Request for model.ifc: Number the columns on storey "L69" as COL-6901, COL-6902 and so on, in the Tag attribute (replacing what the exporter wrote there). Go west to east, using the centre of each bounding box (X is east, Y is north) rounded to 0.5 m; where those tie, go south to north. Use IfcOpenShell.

First a look at what the model holds.

```python
import ifcopenshell
import ifcopenshell.util.element
import ifcopenshell.util.placement

model = ifcopenshell.open("model.ifc")
print(model.schema)
storey = next(s for s in model.by_type("IfcBuildingStorey") if s.Name == "L69")
columns = [e for e in ifcopenshell.util.element.get_decomposition(storey) if e.is_a("IfcColumn")]
for e in sorted(columns, key=lambda e: e.id()):
    origin = ifcopenshell.util.placement.get_local_placement(e.ObjectPlacement)[:3, 3]
    print(e.id(), e.Tag, e.Name, origin.round(2) + 0.0, sep=" | ")
```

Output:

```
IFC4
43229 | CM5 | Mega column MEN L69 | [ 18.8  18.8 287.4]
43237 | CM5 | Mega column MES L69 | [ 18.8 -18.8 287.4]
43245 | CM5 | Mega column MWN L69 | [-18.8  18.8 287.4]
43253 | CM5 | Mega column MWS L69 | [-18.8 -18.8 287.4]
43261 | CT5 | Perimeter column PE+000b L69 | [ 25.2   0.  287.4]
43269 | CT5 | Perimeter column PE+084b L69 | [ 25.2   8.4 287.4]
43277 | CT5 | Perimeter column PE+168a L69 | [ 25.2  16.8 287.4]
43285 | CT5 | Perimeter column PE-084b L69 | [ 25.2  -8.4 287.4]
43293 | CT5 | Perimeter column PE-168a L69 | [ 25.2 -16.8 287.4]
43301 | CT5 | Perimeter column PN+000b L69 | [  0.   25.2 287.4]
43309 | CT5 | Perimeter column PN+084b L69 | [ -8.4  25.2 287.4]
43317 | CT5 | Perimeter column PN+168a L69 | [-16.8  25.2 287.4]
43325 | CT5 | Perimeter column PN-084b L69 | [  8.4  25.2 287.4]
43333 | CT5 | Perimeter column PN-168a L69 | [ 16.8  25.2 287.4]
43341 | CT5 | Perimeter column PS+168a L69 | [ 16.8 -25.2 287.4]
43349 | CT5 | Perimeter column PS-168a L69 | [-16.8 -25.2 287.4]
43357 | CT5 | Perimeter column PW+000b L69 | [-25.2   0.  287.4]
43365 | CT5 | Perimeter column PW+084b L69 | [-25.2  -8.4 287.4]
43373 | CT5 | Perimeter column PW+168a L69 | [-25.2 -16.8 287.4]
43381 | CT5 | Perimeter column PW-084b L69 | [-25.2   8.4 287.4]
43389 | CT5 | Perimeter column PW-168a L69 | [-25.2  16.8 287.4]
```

```python
import ifcopenshell
import ifcopenshell.geom
import ifcopenshell.util.element
import ifcopenshell.util.shape

model = ifcopenshell.open("model.ifc")
settings = ifcopenshell.geom.settings()
settings.set("use-world-coords", True)


def centre(element):
    shape = ifcopenshell.geom.create_shape(settings, element)
    return ifcopenshell.util.shape.get_bbox_centroid(shape.geometry)


storey = next(s for s in model.by_type("IfcBuildingStorey") if s.Name == "L69")
columns = [e for e in ifcopenshell.util.element.get_decomposition(storey) if e.is_a("IfcColumn")]

# Insertion points can sit at a corner or the storey origin, so sort by the geometry (in metres).
centres = {e: centre(e) for e in columns}
columns.sort(key=lambda e: (round(centres[e][0] / 0.5), centres[e][1]))

for i, e in enumerate(columns, start=1):
    number = f"COL-69{i:02d}"
    e.Tag = number
    print(e.id(), number)

model.write("model_v2.ifc")
```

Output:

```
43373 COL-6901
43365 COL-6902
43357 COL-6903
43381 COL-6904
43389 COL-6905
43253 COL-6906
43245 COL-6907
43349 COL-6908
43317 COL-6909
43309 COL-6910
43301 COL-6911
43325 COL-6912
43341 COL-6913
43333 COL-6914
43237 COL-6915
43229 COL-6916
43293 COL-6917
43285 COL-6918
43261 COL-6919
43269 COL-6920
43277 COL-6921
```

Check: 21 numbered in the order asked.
